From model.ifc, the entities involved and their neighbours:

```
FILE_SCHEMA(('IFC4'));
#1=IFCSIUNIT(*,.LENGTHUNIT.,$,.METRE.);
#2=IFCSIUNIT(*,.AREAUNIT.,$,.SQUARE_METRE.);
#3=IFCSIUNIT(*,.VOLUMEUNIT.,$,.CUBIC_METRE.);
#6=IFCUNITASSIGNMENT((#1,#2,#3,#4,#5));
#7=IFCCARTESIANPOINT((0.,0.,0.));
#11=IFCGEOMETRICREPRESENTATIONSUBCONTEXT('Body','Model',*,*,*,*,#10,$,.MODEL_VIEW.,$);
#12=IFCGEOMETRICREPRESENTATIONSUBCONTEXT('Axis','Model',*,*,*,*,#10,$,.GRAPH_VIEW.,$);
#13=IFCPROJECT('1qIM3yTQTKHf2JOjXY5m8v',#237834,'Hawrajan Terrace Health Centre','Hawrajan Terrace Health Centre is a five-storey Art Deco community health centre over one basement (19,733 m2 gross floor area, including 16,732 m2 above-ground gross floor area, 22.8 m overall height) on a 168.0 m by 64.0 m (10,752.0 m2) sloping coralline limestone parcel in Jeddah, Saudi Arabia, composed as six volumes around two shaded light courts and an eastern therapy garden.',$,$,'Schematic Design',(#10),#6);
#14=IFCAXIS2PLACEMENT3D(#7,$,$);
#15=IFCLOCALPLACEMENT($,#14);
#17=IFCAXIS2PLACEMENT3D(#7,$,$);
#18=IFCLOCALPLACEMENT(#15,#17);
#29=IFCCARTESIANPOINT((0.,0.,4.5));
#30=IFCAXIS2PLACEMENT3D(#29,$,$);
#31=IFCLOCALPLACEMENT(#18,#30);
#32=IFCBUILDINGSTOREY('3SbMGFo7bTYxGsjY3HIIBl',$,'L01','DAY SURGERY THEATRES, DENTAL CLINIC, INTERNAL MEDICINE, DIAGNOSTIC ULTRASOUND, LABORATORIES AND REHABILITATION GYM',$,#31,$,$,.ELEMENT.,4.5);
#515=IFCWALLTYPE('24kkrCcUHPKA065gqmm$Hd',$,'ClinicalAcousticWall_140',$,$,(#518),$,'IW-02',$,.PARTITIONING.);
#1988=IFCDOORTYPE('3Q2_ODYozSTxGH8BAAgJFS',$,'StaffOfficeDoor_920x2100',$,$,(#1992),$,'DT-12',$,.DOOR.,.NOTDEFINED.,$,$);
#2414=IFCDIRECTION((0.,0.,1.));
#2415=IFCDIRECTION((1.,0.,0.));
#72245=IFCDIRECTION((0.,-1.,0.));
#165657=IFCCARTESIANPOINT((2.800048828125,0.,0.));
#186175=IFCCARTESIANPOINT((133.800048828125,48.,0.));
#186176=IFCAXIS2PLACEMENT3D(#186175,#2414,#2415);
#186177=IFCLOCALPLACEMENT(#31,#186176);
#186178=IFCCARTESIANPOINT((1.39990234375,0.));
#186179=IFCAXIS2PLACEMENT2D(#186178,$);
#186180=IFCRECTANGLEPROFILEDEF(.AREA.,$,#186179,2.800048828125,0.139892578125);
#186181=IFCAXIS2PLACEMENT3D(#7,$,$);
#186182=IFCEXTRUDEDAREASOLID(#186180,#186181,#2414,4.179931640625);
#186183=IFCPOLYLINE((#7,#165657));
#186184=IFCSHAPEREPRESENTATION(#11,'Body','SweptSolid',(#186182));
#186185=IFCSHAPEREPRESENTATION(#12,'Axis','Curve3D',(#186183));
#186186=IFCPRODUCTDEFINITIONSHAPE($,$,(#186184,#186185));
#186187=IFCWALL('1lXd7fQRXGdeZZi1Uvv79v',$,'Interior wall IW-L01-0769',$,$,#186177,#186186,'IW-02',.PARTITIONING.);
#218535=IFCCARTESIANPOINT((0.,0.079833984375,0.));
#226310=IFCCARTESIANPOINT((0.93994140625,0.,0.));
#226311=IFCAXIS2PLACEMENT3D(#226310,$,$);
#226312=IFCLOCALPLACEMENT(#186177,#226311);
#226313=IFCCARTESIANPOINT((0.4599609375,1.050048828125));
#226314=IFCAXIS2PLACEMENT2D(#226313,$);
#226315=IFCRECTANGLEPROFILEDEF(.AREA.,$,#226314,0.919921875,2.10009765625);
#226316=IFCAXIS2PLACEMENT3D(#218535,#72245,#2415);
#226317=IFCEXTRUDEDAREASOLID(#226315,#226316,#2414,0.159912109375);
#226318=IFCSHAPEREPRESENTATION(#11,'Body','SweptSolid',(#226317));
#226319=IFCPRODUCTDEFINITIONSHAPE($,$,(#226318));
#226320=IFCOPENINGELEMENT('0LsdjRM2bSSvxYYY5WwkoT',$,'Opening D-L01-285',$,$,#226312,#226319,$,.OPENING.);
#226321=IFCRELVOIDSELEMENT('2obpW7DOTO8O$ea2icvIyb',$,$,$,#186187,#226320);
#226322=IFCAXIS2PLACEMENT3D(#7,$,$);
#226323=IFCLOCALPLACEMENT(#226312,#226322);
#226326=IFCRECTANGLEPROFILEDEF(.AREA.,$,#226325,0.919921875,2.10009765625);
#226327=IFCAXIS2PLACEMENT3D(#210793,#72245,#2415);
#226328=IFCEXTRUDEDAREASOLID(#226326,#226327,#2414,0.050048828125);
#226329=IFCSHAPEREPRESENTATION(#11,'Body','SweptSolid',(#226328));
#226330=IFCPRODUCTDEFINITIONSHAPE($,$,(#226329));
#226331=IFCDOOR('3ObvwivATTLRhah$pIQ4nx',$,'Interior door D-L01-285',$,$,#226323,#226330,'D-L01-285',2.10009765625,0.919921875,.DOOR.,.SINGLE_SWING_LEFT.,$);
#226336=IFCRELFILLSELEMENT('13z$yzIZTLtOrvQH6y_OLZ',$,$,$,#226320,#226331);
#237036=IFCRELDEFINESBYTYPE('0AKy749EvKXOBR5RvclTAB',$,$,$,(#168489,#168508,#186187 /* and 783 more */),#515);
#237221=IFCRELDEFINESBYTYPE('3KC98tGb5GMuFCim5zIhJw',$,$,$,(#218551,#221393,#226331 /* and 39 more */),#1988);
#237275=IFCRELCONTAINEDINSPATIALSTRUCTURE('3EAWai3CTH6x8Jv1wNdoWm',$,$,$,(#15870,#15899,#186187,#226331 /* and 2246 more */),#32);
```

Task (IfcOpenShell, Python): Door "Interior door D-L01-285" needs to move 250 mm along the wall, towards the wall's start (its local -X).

```python
import ifcopenshell
import ifcopenshell.api.geometry
import ifcopenshell.util.placement
import ifcopenshell.util.unit

model = ifcopenshell.open("model.ifc")
unit_scale = ifcopenshell.util.unit.calculate_unit_scale(model)

door = model.by_guid("3ObvwivATTLRhah$pIQ4nx")
opening = door.FillsVoids[0].RelatingOpeningElement
wall = opening.VoidsElements[0].RelatingBuildingElement

wall_matrix = ifcopenshell.util.placement.get_local_placement(wall.ObjectPlacement)
shift = wall_matrix[:3, 0] * -0.25 / unit_scale
before = ifcopenshell.util.placement.get_local_placement(door.ObjectPlacement)[:3, 3].copy()

# The door is placed relative to its opening, so it follows when the opening moves.
matrix = ifcopenshell.util.placement.get_local_placement(opening.ObjectPlacement)
matrix[:3, 3] += shift
ifcopenshell.api.geometry.edit_object_placement(
    model, product=opening, matrix=matrix, is_si=False, should_transform_children=True
)

after = ifcopenshell.util.placement.get_local_placement(door.ObjectPlacement)[:3, 3]
print("door moved by", (after - before).round(3) + 0.0)

model.write("model_v2.ifc")
```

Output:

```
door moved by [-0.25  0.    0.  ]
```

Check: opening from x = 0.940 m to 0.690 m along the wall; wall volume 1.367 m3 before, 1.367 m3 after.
